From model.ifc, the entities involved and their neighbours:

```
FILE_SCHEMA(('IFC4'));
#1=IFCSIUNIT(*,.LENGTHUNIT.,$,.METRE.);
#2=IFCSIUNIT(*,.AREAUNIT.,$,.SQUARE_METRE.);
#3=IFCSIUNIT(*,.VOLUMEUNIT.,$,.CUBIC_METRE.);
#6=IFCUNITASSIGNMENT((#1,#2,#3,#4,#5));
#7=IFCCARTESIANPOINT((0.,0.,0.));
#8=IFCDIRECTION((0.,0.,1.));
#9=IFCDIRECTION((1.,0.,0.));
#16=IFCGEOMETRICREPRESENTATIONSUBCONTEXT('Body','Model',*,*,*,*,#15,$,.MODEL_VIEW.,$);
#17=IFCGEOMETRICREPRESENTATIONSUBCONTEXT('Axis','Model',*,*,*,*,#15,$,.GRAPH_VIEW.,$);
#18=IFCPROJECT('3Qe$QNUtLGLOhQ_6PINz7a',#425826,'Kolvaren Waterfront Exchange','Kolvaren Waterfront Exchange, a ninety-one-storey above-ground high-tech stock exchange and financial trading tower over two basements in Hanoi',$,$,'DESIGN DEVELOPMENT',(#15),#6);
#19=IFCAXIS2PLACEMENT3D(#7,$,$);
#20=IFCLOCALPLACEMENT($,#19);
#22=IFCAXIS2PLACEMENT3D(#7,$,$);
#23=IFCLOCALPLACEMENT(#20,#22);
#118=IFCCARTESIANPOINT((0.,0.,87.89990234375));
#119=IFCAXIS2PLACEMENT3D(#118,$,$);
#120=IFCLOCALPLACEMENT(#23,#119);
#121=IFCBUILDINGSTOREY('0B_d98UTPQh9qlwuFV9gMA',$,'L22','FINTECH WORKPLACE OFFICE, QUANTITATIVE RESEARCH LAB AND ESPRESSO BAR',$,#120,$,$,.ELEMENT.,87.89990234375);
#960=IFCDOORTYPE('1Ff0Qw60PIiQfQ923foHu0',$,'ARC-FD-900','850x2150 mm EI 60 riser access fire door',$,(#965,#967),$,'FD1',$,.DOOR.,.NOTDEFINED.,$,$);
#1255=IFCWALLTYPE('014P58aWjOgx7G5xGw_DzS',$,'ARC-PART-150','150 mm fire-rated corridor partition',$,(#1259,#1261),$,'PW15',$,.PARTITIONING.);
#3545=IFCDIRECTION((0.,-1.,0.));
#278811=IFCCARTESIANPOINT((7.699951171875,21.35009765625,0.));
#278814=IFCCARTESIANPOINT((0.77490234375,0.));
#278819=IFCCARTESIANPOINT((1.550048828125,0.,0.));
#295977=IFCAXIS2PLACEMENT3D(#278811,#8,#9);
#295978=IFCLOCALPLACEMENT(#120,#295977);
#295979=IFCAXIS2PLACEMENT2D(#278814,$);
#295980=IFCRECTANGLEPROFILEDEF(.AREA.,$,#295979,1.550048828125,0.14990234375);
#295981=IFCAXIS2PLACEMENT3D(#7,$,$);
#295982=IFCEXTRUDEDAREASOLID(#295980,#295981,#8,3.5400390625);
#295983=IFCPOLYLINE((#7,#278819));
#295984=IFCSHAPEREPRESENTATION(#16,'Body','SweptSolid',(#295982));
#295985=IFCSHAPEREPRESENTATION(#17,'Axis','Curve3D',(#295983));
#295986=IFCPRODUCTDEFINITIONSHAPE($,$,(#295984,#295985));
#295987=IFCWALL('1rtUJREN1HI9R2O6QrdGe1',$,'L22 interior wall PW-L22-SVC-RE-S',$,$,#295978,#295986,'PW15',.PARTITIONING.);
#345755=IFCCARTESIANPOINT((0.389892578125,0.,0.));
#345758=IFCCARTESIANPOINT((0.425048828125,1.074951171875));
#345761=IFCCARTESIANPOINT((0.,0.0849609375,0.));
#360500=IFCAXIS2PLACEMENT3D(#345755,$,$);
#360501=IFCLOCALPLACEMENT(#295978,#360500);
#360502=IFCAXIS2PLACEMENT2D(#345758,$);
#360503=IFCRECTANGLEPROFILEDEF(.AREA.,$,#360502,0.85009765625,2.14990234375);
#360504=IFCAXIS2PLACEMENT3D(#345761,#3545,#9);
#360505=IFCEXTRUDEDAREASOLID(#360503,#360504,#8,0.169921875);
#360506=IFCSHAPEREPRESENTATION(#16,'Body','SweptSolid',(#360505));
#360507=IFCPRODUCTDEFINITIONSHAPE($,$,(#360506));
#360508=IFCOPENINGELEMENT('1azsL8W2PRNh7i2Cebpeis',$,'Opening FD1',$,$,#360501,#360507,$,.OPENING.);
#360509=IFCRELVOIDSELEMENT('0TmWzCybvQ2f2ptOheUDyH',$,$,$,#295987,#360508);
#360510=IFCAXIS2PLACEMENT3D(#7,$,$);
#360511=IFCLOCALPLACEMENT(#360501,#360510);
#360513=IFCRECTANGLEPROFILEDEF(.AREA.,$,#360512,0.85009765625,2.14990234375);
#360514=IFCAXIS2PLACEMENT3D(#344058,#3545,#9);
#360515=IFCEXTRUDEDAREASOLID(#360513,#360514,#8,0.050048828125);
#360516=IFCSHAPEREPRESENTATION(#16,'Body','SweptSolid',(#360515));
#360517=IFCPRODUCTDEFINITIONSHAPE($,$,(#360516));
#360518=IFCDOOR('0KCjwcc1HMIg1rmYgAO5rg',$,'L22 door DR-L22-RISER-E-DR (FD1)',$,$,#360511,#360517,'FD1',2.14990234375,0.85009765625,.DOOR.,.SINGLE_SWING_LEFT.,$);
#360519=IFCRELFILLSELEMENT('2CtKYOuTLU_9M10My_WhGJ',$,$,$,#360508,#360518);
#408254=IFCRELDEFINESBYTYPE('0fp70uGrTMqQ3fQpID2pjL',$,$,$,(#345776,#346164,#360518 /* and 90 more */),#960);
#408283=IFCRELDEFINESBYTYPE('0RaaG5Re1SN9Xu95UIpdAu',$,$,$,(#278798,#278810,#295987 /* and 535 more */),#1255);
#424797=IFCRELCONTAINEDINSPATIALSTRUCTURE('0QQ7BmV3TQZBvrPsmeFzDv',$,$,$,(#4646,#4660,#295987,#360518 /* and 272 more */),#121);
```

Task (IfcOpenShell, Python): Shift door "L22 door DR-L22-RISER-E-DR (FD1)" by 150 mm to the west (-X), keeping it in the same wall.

```python
import ifcopenshell
import ifcopenshell.api.geometry
import ifcopenshell.util.placement
import ifcopenshell.util.unit

model = ifcopenshell.open("model.ifc")
unit_scale = ifcopenshell.util.unit.calculate_unit_scale(model)

door = model.by_guid("0KCjwcc1HMIg1rmYgAO5rg")
opening = door.FillsVoids[0].RelatingOpeningElement
wall = opening.VoidsElements[0].RelatingBuildingElement

wall_matrix = ifcopenshell.util.placement.get_local_placement(wall.ObjectPlacement)
shift = wall_matrix[:3, 0] * -0.15 / unit_scale
before = ifcopenshell.util.placement.get_local_placement(door.ObjectPlacement)[:3, 3].copy()

# The door is placed relative to its opening, so it follows when the opening moves.
matrix = ifcopenshell.util.placement.get_local_placement(opening.ObjectPlacement)
matrix[:3, 3] += shift
ifcopenshell.api.geometry.edit_object_placement(
    model, product=opening, matrix=matrix, is_si=False, should_transform_children=True
)

after = ifcopenshell.util.placement.get_local_placement(door.ObjectPlacement)[:3, 3]
print("door moved by", (after - before).round(3) + 0.0)

model.write("model_v2.ifc")
```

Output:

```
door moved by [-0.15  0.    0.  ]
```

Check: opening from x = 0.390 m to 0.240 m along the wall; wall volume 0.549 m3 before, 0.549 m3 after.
